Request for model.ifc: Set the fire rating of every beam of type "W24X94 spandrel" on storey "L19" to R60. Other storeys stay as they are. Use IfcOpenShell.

First a look at what the model holds.

```python
import ifcopenshell
import ifcopenshell.util.element

model = ifcopenshell.open("model.ifc")
print(model.schema)
storey = next(s for s in model.by_type("IfcBuildingStorey") if s.Name == "L19")
beams = [e for e in ifcopenshell.util.element.get_decomposition(storey) if e.is_a("IfcBeam")]
seen = {}
for e in beams:
    element_type = ifcopenshell.util.element.get_type(e)
    key = (element_type.Name if element_type != e and element_type else None, ifcopenshell.util.element.get_pset(e, "Pset_BeamCommon", "FireRating"))
    seen[key] = seen.get(key, 0) + 1
for (name, value), count in sorted(seen.items(), key=str):
    print(count, "x", name, "|", value)
```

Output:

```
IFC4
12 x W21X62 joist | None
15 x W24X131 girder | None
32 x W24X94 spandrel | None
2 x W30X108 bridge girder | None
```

```python
import ifcopenshell
import ifcopenshell.api.pset
import ifcopenshell.util.element

model = ifcopenshell.open("model.ifc")

storey = next(s for s in model.by_type("IfcBuildingStorey") if s.Name == "L19")
beams = [e for e in ifcopenshell.util.element.get_decomposition(storey) if e.is_a("IfcBeam")]

count = 0
for e in beams:
    element_type = ifcopenshell.util.element.get_type(e)
    if element_type in (None, e) or element_type.Name != "W24X94 spandrel":
        continue
    found = ifcopenshell.util.element.get_pset(e, "Pset_BeamCommon", should_inherit=False)
    if found:
        pset = model.by_id(found["id"])
        if len(ifcopenshell.util.element.get_elements_by_pset(pset)) > 1:
            pset = ifcopenshell.api.pset.unshare_pset(model, products=[e], pset=pset)[0]
    else:
        pset = ifcopenshell.api.pset.add_pset(model, product=e, name="Pset_BeamCommon")
    ifcopenshell.api.pset.edit_pset(model, pset=pset, properties={"FireRating": "R60"})
    count += 1

print(count, "beams updated")

model.write("model_rev.ifc")
```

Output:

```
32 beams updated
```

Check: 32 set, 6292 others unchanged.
